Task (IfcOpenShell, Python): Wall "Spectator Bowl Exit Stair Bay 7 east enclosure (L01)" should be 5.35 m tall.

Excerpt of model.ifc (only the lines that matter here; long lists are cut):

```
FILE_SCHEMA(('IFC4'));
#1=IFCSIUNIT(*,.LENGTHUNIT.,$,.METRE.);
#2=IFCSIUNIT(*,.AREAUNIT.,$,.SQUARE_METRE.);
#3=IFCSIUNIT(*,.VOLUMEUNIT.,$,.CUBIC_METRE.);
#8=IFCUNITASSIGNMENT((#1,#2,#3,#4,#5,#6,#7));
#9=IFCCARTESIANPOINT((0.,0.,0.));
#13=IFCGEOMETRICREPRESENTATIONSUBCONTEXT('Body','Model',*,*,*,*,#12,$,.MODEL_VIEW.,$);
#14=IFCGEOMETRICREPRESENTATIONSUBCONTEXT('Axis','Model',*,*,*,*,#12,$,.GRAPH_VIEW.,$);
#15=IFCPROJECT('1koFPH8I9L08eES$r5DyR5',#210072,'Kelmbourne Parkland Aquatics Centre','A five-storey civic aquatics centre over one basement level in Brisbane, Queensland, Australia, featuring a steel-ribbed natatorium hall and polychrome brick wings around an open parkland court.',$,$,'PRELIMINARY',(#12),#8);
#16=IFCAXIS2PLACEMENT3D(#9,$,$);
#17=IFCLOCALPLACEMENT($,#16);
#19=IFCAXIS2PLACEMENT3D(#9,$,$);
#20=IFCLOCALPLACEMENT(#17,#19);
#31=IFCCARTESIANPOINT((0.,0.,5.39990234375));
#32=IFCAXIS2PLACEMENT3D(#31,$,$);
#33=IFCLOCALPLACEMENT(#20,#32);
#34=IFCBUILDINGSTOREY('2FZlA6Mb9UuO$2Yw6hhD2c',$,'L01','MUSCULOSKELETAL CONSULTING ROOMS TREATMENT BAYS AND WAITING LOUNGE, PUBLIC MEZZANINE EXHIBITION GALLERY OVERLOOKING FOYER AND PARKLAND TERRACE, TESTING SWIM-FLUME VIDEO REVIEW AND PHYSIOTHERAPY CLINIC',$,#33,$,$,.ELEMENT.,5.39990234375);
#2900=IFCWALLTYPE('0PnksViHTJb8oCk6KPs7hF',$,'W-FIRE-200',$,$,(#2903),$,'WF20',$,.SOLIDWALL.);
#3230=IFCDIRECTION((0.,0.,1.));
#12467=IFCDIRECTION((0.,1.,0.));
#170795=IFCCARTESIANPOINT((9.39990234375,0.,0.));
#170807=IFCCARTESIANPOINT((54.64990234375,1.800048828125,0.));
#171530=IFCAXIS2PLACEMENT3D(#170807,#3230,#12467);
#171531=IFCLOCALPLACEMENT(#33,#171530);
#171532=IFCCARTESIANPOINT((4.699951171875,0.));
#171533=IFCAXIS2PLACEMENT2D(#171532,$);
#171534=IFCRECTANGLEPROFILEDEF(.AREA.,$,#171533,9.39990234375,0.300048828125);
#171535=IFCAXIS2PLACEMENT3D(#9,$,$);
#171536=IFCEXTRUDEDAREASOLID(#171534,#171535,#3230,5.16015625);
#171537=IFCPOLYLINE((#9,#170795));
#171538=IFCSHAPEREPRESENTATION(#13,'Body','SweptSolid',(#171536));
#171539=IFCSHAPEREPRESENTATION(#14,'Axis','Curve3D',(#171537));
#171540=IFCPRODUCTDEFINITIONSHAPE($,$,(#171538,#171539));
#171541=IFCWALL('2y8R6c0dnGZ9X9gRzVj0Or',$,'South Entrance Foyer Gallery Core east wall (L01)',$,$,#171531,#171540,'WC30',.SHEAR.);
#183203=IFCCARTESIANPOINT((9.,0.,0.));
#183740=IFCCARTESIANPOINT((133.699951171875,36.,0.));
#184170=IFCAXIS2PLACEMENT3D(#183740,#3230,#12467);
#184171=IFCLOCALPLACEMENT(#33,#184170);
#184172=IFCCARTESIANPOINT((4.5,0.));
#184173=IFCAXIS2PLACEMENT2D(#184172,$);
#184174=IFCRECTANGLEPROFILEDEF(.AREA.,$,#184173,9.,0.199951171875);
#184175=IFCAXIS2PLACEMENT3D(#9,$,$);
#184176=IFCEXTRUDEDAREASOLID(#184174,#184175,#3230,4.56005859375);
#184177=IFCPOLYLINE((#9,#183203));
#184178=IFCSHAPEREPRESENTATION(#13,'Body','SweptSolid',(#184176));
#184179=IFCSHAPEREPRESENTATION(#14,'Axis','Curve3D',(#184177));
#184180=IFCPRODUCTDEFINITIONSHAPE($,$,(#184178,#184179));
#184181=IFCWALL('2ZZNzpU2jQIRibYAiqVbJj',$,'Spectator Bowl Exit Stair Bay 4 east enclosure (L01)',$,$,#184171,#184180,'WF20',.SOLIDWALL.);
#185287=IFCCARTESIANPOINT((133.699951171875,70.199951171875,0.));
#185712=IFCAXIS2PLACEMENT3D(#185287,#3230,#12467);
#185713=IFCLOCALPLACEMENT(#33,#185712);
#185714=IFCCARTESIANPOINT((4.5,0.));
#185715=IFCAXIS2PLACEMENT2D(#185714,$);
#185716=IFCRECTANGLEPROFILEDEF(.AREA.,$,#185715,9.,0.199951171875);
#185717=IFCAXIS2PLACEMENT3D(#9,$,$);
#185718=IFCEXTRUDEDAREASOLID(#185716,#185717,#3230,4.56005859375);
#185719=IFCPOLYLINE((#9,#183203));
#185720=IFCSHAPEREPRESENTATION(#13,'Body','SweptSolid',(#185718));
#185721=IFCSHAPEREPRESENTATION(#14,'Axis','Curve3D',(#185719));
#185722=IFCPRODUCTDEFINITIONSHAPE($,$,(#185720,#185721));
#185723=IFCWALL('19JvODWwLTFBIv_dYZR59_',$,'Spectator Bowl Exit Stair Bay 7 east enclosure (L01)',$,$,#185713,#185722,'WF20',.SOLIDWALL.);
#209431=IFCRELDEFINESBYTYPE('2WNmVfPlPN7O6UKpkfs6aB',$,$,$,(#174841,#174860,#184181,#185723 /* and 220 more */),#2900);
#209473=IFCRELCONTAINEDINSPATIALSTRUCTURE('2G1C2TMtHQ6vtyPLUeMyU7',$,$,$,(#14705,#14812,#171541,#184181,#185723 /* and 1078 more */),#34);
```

```python
import ifcopenshell
import ifcopenshell.geom
import ifcopenshell.util.representation
import ifcopenshell.util.shape
import ifcopenshell.util.unit

model = ifcopenshell.open("model.ifc")
unit_scale = ifcopenshell.util.unit.calculate_unit_scale(model)
settings = ifcopenshell.geom.settings()


def volume(element):
    """Net volume in cubic metres, openings subtracted."""
    shape = ifcopenshell.geom.create_shape(settings, element)
    return ifcopenshell.util.shape.get_volume(shape.geometry)


wall = model.by_id(185723)
before = volume(wall)

body = ifcopenshell.util.representation.get_representation(wall, "Model", "Body")
solid = body.Items[0]
old_height = solid.Depth
solid.Depth = 5.35 / unit_scale
after = volume(wall)

print(f"height {old_height:g} -> {solid.Depth:g}, volume {before:.3f} -> {after:.3f} m3")

model.write("model_v2.ifc")
```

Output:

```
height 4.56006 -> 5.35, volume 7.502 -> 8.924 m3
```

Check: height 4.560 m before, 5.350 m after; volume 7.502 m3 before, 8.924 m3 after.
